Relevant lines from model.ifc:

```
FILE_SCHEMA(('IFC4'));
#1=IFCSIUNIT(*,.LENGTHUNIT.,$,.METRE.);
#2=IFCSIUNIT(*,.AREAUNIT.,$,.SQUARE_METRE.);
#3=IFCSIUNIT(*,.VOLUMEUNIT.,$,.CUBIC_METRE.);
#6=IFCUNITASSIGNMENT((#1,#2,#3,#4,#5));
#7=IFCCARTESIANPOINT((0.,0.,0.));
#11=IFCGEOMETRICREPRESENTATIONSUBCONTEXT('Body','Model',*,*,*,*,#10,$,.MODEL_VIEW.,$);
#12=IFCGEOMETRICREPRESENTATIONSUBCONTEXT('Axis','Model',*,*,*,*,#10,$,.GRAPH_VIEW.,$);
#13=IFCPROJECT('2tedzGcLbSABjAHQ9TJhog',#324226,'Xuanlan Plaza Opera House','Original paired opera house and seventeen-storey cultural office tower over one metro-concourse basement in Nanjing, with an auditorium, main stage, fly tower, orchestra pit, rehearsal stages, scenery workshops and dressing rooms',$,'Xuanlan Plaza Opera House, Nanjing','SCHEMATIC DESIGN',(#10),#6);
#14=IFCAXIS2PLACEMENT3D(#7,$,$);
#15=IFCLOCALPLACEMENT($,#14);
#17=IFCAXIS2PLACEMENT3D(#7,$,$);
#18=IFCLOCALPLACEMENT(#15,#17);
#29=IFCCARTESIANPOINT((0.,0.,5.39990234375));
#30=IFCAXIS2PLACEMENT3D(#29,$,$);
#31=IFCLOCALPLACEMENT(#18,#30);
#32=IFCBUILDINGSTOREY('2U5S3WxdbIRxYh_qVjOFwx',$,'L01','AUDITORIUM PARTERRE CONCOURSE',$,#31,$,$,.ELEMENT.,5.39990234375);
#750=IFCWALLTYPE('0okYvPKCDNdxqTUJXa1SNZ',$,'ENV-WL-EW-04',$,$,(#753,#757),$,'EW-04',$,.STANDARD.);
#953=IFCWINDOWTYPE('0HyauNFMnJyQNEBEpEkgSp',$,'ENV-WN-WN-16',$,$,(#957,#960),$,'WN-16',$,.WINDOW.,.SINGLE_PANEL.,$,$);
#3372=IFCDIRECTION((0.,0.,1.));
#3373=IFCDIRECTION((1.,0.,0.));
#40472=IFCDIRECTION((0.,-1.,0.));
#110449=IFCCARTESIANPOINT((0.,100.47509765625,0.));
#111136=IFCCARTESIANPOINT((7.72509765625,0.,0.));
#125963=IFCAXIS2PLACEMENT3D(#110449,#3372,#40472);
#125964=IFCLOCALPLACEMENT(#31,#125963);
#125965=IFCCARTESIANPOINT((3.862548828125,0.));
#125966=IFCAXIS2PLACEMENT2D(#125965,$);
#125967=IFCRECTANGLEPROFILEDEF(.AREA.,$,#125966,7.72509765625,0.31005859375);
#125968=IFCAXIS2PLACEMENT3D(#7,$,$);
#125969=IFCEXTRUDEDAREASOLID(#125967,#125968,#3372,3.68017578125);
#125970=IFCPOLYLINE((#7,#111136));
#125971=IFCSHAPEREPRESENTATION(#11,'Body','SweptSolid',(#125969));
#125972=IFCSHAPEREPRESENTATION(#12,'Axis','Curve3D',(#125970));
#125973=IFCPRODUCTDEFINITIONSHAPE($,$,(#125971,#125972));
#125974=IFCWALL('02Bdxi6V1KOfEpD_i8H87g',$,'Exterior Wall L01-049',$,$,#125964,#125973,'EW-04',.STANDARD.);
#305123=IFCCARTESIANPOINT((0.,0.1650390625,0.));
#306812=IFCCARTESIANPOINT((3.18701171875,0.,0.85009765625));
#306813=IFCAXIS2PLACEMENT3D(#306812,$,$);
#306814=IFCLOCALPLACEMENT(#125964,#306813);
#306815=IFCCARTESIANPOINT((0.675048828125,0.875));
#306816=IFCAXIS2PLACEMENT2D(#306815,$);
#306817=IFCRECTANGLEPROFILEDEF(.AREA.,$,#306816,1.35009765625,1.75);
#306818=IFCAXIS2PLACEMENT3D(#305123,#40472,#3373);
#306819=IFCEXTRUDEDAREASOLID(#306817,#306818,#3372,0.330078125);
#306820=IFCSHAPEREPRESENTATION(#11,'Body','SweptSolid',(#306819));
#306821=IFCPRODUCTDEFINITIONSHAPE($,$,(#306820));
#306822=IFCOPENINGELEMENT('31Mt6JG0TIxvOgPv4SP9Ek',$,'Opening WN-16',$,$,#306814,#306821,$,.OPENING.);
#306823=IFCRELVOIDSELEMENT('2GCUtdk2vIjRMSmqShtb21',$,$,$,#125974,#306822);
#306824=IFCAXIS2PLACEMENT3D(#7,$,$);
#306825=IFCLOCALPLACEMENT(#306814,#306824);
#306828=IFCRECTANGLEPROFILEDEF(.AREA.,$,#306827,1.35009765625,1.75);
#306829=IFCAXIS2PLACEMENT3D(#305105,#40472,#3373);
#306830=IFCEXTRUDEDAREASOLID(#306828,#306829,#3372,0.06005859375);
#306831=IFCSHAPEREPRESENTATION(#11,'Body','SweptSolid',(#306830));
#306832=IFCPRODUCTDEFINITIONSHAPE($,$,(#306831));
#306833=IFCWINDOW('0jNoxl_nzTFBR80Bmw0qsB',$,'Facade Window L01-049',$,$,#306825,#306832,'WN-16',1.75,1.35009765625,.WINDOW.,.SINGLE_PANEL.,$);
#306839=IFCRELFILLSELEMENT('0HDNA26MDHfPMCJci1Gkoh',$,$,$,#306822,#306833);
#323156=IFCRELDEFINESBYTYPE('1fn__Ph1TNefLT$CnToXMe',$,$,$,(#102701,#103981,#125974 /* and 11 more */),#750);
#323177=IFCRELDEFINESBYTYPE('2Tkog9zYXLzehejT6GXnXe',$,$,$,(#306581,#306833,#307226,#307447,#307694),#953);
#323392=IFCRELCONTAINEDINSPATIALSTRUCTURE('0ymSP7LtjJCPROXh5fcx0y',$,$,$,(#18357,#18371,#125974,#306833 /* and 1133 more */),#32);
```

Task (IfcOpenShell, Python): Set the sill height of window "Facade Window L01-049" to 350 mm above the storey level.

```python
import numpy as np
import ifcopenshell
import ifcopenshell.api.geometry
import ifcopenshell.geom
import ifcopenshell.util.element
import ifcopenshell.util.placement
import ifcopenshell.util.shape
import ifcopenshell.util.unit

model = ifcopenshell.open("model.ifc")
unit_scale = ifcopenshell.util.unit.calculate_unit_scale(model)

window = model.by_guid("0jNoxl_nzTFBR80Bmw0qsB")
opening = window.FillsVoids[0].RelatingOpeningElement
storey = ifcopenshell.util.element.get_container(window, ifc_class="IfcBuildingStorey")
level = ifcopenshell.util.placement.get_local_placement(storey.ObjectPlacement)[2, 3]

# The opening's origin need not be at the sill, so measure its lowest point.
shape = ifcopenshell.geom.create_shape(ifcopenshell.geom.settings(), opening)
bottom = ifcopenshell.util.shape.get_shape_bottom_elevation(shape, shape.geometry) / unit_scale
dz = level + 0.35 / unit_scale - bottom

shift = np.array([0.0, 0.0, dz])
# The window is placed relative to its opening, so it follows when the opening moves.
matrix = ifcopenshell.util.placement.get_local_placement(opening.ObjectPlacement)
matrix[:3, 3] += shift
ifcopenshell.api.geometry.edit_object_placement(
    model, product=opening, matrix=matrix, is_si=False, should_transform_children=True
)

print(f"moved by {dz * unit_scale:+.3f} m")

model.write("model_rev.ifc")
```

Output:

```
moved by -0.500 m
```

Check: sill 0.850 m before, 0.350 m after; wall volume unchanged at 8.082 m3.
